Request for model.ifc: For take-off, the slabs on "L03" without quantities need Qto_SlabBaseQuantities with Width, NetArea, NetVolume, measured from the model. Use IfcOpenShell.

First a look at what the model holds.

```python
import ifcopenshell
import ifcopenshell.util.element
import ifcopenshell.util.unit

model = ifcopenshell.open("model.ifc")
print(model.schema)
for unit_type in ("LENGTHUNIT", "AREAUNIT", "VOLUMEUNIT"):
    print(unit_type, ifcopenshell.util.unit.calculate_unit_scale(model, unit_type))
storey = next(s for s in model.by_type("IfcBuildingStorey") if s.Name == "L03")
slabs = [e for e in ifcopenshell.util.element.get_decomposition(storey) if e.is_a("IfcSlab")]
for e in sorted(slabs, key=lambda e: e.id()):
    print(e.id(), e.is_a(), e.Name, list(ifcopenshell.util.element.get_psets(e, qtos_only=True)), sep=" | ")
```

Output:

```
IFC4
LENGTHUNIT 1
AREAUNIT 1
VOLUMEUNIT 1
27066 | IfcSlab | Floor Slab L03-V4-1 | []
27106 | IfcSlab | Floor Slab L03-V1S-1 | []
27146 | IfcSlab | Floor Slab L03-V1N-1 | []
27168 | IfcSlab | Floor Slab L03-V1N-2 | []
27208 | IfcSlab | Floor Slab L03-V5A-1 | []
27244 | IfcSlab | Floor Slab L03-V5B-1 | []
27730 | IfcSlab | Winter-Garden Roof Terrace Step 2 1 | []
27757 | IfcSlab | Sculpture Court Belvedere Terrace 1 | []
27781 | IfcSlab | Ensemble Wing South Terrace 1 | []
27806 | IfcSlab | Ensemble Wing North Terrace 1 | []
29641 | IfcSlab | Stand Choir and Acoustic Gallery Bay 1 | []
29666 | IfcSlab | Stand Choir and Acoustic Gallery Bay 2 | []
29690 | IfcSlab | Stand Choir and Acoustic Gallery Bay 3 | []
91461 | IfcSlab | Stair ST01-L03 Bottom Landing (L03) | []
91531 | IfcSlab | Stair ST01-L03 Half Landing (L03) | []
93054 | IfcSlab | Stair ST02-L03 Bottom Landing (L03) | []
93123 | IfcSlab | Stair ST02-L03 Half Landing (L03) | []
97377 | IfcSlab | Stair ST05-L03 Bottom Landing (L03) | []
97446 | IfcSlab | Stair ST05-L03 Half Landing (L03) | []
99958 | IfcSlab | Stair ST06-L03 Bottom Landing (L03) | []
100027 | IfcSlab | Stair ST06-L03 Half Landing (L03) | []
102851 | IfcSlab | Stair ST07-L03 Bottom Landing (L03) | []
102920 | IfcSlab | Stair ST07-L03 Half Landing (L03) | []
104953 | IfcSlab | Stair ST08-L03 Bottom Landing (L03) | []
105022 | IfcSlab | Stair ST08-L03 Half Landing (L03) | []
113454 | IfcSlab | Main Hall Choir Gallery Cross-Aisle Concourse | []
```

```python
import ifcopenshell
import ifcopenshell.api.pset
import ifcopenshell.geom
import ifcopenshell.util.element
import ifcopenshell.util.shape
import ifcopenshell.util.unit

model = ifcopenshell.open("model.ifc")
unit_scale = ifcopenshell.util.unit.calculate_unit_scale(model)
area_scale = ifcopenshell.util.unit.calculate_unit_scale(model, "AREAUNIT")
volume_scale = ifcopenshell.util.unit.calculate_unit_scale(model, "VOLUMEUNIT")
settings = ifcopenshell.geom.settings()

storey = next(s for s in model.by_type("IfcBuildingStorey") if s.Name == "L03")
slabs = [e for e in ifcopenshell.util.element.get_decomposition(storey) if e.is_a("IfcSlab")]

for e in sorted(slabs, key=lambda e: e.id()):
    if ifcopenshell.util.element.get_psets(e, qtos_only=True, should_inherit=False):
        continue
    # Geometry comes back in metres, in the element's own axes.
    shape = ifcopenshell.geom.create_shape(settings, e)
    values = {
        "Width": ifcopenshell.util.shape.get_z(shape.geometry) / unit_scale,
        "NetArea": ifcopenshell.util.shape.get_footprint_area(shape.geometry) / area_scale,
        "NetVolume": ifcopenshell.util.shape.get_volume(shape.geometry) / volume_scale,
    }
    qto = ifcopenshell.api.pset.add_qto(model, product=e, name="Qto_SlabBaseQuantities")
    ifcopenshell.api.pset.edit_qto(model, qto=qto, properties=values)
    print(e.id(), {k: round(v, 3) for k, v in values.items()})

model.write("model_rev.ifc")
```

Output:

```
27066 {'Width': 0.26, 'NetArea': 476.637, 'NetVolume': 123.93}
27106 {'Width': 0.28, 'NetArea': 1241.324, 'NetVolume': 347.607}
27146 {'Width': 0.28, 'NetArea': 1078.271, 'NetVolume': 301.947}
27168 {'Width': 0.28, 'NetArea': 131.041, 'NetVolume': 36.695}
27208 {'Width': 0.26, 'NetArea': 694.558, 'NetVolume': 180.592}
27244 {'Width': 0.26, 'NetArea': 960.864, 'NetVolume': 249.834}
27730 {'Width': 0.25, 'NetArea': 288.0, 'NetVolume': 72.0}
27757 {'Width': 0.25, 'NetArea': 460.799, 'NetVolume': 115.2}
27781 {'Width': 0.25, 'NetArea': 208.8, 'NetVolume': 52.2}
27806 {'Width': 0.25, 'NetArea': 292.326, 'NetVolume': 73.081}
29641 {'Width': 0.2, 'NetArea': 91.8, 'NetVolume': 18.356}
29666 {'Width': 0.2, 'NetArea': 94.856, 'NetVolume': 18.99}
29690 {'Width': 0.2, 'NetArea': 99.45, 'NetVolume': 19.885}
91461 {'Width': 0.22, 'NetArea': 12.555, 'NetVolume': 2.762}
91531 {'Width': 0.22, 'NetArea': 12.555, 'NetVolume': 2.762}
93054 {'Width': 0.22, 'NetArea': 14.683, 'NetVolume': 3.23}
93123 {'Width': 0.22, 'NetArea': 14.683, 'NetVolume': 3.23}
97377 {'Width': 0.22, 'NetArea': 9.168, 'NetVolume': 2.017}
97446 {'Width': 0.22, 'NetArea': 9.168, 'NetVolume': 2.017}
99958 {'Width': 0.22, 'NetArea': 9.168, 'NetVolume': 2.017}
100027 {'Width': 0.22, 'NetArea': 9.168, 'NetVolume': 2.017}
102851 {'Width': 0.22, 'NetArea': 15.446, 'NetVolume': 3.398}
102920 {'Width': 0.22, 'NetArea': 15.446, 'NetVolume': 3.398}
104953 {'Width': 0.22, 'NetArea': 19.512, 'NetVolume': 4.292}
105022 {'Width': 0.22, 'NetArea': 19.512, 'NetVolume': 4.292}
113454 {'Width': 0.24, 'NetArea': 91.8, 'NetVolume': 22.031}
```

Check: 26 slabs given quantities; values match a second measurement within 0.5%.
